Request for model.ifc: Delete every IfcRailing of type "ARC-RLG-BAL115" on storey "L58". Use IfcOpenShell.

First a look at what the model holds.

```python
import ifcopenshell
import ifcopenshell.util.element

model = ifcopenshell.open("model.ifc")
print(model.schema)
storey = next(s for s in model.by_type("IfcBuildingStorey") if s.Name == "L58")
railings = [e for e in ifcopenshell.util.element.get_decomposition(storey) if e.is_a("IfcRailing")]
seen = {}
for e in railings:
    element_type = ifcopenshell.util.element.get_type(e)
    name = element_type.Name if element_type not in (None, e) else None
    seen[name] = seen.get(name, 0) + 1
for name, count in sorted(seen.items(), key=str):
    print(count, "x", name)
```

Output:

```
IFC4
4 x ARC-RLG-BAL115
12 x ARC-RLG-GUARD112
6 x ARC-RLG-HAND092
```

```python
import ifcopenshell
import ifcopenshell.api.root
import ifcopenshell.util.element

model = ifcopenshell.open("model.ifc")

storey = next(s for s in model.by_type("IfcBuildingStorey") if s.Name == "L58")
railings = [e for e in ifcopenshell.util.element.get_decomposition(storey) if e.is_a("IfcRailing")]
targets = [e for e in railings if (t := ifcopenshell.util.element.get_type(e)) not in (None, e) and t.Name == "ARC-RLG-BAL115"]

for e in targets:
    ifcopenshell.api.root.remove_product(model, product=e)
print(len(targets), "removed")

model.write("model-out.ifc")
```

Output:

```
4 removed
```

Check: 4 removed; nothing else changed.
